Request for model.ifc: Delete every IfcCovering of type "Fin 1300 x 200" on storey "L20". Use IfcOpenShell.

First a look at what the model holds.

```python
import ifcopenshell
import ifcopenshell.util.element

model = ifcopenshell.open("model.ifc")
print(model.schema)
storey = next(s for s in model.by_type("IfcBuildingStorey") if s.Name == "L20")
coverings = [e for e in ifcopenshell.util.element.get_decomposition(storey) if e.is_a("IfcCovering")]
seen = {}
for e in coverings:
    element_type = ifcopenshell.util.element.get_type(e)
    name = element_type.Name if element_type not in (None, e) else None
    seen[name] = seen.get(name, 0) + 1
for name, count in sorted(seen.items(), key=str):
    print(count, "x", name)
```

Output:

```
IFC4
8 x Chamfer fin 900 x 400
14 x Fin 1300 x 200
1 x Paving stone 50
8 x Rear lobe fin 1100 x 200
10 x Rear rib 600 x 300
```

```python
import ifcopenshell
import ifcopenshell.api.root
import ifcopenshell.util.element

model = ifcopenshell.open("model.ifc")

storey = next(s for s in model.by_type("IfcBuildingStorey") if s.Name == "L20")
coverings = [e for e in ifcopenshell.util.element.get_decomposition(storey) if e.is_a("IfcCovering")]
targets = [e for e in coverings if (t := ifcopenshell.util.element.get_type(e)) not in (None, e) and t.Name == "Fin 1300 x 200"]

for e in targets:
    ifcopenshell.api.root.remove_product(model, product=e)
print(len(targets), "removed")

model.write("model_v2.ifc")
```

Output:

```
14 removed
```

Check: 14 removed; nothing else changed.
